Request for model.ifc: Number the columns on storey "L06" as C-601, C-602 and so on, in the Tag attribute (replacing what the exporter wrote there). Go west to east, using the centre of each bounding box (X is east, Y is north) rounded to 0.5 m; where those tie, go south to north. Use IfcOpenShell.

First a look at what the model holds.

```python
import ifcopenshell
import ifcopenshell.util.element
import ifcopenshell.util.placement

model = ifcopenshell.open("model.ifc")
print(model.schema)
storey = next(s for s in model.by_type("IfcBuildingStorey") if s.Name == "L06")
columns = [e for e in ifcopenshell.util.element.get_decomposition(storey) if e.is_a("IfcColumn")]
for e in sorted(columns, key=lambda e: e.id()):
    origin = ifcopenshell.util.placement.get_local_placement(e.ObjectPlacement)[:3, 3]
    print(e.id(), e.Tag, e.Name, origin.round(2) + 0.0, sep=" | ")
```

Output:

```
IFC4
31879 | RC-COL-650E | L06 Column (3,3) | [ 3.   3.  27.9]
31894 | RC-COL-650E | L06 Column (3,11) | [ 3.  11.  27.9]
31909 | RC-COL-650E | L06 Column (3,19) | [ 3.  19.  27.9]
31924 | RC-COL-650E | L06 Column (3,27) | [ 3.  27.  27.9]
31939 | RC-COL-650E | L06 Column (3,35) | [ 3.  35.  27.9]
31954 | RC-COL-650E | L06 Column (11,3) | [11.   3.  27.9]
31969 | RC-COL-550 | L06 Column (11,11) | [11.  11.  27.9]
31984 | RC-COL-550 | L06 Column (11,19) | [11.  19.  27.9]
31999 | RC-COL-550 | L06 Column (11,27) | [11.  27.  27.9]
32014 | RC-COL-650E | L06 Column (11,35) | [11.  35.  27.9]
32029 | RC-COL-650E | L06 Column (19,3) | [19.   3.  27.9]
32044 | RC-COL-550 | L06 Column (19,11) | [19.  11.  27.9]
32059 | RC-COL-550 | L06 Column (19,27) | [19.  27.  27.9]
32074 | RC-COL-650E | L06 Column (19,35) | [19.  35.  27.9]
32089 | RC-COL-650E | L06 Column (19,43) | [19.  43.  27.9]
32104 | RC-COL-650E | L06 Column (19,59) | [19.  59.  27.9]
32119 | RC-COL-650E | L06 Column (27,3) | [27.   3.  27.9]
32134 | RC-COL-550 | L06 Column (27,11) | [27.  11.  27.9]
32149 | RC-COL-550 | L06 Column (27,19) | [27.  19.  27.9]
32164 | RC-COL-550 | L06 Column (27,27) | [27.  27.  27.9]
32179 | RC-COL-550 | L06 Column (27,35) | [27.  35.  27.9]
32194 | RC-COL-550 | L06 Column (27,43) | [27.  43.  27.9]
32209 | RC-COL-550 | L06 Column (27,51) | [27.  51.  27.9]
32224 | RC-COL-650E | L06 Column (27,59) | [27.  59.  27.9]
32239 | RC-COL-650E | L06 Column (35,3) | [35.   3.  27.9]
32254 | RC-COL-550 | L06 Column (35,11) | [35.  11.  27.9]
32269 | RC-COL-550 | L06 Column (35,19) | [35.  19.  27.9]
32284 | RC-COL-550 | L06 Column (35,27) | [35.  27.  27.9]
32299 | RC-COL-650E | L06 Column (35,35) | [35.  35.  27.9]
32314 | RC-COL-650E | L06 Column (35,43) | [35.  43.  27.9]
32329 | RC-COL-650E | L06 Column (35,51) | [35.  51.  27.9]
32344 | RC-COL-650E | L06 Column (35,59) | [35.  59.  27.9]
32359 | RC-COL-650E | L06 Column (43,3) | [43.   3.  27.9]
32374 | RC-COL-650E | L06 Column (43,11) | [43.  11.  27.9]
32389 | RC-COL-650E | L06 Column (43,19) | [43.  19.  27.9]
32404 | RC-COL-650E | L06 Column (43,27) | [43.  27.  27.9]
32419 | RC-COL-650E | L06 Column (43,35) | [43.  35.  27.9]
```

```python
import ifcopenshell
import ifcopenshell.geom
import ifcopenshell.util.element
import ifcopenshell.util.shape

model = ifcopenshell.open("model.ifc")
settings = ifcopenshell.geom.settings()
settings.set("use-world-coords", True)


def centre(element):
    shape = ifcopenshell.geom.create_shape(settings, element)
    return ifcopenshell.util.shape.get_bbox_centroid(shape.geometry)


storey = next(s for s in model.by_type("IfcBuildingStorey") if s.Name == "L06")
columns = [e for e in ifcopenshell.util.element.get_decomposition(storey) if e.is_a("IfcColumn")]

# Insertion points can sit at a corner or the storey origin, so sort by the geometry (in metres).
centres = {e: centre(e) for e in columns}
columns.sort(key=lambda e: (round(centres[e][0] / 0.5), centres[e][1]))

for i, e in enumerate(columns, start=1):
    number = f"C-6{i:02d}"
    e.Tag = number
    print(e.id(), number)

model.write("model-out.ifc")
```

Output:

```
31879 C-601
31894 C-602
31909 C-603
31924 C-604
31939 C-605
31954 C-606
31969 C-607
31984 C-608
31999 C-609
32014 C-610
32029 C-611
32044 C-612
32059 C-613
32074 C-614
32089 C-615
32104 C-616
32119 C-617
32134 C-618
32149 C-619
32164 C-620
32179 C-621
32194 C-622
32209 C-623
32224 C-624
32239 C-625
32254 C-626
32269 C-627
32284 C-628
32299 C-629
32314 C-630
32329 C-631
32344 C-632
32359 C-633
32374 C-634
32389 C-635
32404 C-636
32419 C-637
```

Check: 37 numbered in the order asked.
